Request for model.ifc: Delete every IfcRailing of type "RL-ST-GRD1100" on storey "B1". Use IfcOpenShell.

First a look at what the model holds.

```python
import ifcopenshell
import ifcopenshell.util.element

model = ifcopenshell.open("model.ifc")
print(model.schema)
storey = next(s for s in model.by_type("IfcBuildingStorey") if s.Name == "B1")
railings = [e for e in ifcopenshell.util.element.get_decomposition(storey) if e.is_a("IfcRailing")]
seen = {}
for e in railings:
    element_type = ifcopenshell.util.element.get_type(e)
    name = element_type.Name if element_type not in (None, e) else None
    seen[name] = seen.get(name, 0) + 1
for name, count in sorted(seen.items(), key=str):
    print(count, "x", name)
```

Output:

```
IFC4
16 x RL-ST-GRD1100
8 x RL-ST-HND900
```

```python
import ifcopenshell
import ifcopenshell.api.root
import ifcopenshell.util.element

model = ifcopenshell.open("model.ifc")

storey = next(s for s in model.by_type("IfcBuildingStorey") if s.Name == "B1")
railings = [e for e in ifcopenshell.util.element.get_decomposition(storey) if e.is_a("IfcRailing")]
targets = [e for e in railings if (t := ifcopenshell.util.element.get_type(e)) not in (None, e) and t.Name == "RL-ST-GRD1100"]

for e in targets:
    ifcopenshell.api.root.remove_product(model, product=e)
print(len(targets), "removed")

model.write("model_v2.ifc")
```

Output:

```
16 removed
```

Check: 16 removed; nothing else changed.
